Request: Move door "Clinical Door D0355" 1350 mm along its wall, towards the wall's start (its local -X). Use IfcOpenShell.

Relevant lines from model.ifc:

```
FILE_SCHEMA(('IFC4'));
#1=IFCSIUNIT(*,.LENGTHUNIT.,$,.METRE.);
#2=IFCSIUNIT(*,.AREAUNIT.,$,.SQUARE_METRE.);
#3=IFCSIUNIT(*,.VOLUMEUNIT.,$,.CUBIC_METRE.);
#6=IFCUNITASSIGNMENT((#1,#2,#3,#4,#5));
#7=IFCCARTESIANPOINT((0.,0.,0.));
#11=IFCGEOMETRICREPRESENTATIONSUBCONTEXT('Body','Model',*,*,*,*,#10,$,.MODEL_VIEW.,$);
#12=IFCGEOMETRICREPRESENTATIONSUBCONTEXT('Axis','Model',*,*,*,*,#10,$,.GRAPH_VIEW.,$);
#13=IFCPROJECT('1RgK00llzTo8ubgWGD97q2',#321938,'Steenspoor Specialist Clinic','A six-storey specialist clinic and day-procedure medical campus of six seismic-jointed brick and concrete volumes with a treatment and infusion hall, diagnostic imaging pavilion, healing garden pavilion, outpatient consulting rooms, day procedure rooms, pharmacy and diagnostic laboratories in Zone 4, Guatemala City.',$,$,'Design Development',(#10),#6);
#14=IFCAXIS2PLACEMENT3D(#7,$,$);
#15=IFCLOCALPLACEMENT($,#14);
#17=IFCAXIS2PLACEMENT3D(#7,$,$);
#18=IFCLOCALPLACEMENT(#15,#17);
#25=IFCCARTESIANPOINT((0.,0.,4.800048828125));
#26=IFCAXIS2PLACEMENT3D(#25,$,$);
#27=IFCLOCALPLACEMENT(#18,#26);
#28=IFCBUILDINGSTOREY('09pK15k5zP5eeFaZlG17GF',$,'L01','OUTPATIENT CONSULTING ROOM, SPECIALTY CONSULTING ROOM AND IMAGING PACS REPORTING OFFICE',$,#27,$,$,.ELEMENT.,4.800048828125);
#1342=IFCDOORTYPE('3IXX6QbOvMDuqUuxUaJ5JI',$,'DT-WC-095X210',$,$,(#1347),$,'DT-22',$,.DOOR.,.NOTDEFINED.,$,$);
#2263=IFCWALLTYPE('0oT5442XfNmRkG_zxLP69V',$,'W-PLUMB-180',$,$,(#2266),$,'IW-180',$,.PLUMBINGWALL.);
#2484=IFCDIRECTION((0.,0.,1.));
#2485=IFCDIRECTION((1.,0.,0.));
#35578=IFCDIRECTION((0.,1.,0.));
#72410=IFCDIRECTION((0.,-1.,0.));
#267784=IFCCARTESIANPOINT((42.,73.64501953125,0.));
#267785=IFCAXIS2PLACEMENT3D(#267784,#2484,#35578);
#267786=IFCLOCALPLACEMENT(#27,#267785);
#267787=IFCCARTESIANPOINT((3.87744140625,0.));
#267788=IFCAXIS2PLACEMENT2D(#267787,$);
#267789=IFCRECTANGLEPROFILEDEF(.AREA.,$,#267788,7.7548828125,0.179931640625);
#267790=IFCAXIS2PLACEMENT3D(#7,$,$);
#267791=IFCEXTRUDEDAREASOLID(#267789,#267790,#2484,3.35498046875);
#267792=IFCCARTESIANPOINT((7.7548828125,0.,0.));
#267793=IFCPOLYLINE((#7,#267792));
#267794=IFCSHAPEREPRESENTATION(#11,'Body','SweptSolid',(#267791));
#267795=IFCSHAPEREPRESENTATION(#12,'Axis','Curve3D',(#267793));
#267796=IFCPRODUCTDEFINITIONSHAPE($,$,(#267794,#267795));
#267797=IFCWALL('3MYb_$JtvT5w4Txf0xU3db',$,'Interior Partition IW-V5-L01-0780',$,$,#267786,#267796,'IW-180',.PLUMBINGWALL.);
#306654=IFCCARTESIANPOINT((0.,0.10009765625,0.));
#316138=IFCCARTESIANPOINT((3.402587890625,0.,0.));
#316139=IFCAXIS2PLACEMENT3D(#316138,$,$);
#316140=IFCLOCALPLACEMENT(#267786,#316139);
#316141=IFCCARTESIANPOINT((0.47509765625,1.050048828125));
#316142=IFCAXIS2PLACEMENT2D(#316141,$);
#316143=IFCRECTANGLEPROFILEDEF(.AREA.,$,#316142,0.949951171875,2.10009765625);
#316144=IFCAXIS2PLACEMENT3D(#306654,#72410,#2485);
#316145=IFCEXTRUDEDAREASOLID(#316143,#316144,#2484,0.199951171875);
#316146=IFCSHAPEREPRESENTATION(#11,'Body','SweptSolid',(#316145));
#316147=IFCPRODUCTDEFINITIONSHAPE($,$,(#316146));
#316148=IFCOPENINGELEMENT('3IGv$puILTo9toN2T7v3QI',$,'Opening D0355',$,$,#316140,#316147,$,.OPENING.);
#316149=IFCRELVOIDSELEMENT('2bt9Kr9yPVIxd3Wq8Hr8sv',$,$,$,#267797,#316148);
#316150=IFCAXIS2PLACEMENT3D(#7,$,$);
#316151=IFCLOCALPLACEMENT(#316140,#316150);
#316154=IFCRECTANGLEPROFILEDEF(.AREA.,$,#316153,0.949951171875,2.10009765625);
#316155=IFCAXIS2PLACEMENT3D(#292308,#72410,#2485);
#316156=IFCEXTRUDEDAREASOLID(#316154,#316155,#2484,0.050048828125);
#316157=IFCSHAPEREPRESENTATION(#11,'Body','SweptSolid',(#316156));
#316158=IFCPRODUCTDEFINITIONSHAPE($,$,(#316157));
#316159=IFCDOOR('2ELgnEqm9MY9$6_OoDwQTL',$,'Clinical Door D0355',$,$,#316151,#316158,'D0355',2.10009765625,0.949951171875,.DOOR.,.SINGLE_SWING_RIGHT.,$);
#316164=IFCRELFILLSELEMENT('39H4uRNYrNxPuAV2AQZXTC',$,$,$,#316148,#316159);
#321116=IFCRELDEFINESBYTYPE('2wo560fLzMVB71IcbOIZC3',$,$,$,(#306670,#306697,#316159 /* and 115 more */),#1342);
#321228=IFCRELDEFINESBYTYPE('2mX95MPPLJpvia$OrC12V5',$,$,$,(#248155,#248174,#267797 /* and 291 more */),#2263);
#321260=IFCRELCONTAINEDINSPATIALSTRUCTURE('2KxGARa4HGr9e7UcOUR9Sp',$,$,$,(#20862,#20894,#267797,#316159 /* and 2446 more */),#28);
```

```python
import ifcopenshell
import ifcopenshell.api.geometry
import ifcopenshell.util.placement
import ifcopenshell.util.unit

model = ifcopenshell.open("model.ifc")
unit_scale = ifcopenshell.util.unit.calculate_unit_scale(model)

door = model.by_id(316159)
opening = door.FillsVoids[0].RelatingOpeningElement
wall = opening.VoidsElements[0].RelatingBuildingElement

wall_matrix = ifcopenshell.util.placement.get_local_placement(wall.ObjectPlacement)
shift = wall_matrix[:3, 0] * -1.35 / unit_scale
before = ifcopenshell.util.placement.get_local_placement(door.ObjectPlacement)[:3, 3].copy()

# The door is placed relative to its opening, so it follows when the opening moves.
matrix = ifcopenshell.util.placement.get_local_placement(opening.ObjectPlacement)
matrix[:3, 3] += shift
ifcopenshell.api.geometry.edit_object_placement(
    model, product=opening, matrix=matrix, is_si=False, should_transform_children=True
)

after = ifcopenshell.util.placement.get_local_placement(door.ObjectPlacement)[:3, 3]
print("door moved by", (after - before).round(3) + 0.0)

model.write("model_updated.ifc")
```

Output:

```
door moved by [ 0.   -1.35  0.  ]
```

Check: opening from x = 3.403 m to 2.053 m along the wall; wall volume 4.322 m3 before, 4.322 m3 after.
